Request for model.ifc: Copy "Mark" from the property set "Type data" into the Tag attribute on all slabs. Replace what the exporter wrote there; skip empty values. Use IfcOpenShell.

First a look at what the model holds.

```python
import ifcopenshell
import ifcopenshell.util.element

model = ifcopenshell.open("model.ifc")
print(model.schema)
slabs = model.by_type("IfcSlab")
print(len(slabs), "slabs")
for e in slabs[:8]:
    source = ifcopenshell.util.element.get_pset(e, "Type data", "Mark")
    target = e.Tag
    print(e.id(), repr(source), repr(target), sep=" | ")
```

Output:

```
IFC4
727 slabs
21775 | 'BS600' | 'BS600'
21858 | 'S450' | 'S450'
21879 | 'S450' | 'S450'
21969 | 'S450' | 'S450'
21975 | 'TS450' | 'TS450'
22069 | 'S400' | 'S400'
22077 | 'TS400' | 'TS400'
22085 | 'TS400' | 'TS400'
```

```python
import ifcopenshell
import ifcopenshell.util.element

model = ifcopenshell.open("model.ifc")

count = 0
for e in model.by_type("IfcSlab"):
    value = ifcopenshell.util.element.get_pset(e, "Type data", "Mark")
    current = e.Tag
    if not value or not value.strip() or current == value:
        continue
    e.Tag = value
    count += 1

print(count, "slabs updated")

model.write("model-out.ifc")
```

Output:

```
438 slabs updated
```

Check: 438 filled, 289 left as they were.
